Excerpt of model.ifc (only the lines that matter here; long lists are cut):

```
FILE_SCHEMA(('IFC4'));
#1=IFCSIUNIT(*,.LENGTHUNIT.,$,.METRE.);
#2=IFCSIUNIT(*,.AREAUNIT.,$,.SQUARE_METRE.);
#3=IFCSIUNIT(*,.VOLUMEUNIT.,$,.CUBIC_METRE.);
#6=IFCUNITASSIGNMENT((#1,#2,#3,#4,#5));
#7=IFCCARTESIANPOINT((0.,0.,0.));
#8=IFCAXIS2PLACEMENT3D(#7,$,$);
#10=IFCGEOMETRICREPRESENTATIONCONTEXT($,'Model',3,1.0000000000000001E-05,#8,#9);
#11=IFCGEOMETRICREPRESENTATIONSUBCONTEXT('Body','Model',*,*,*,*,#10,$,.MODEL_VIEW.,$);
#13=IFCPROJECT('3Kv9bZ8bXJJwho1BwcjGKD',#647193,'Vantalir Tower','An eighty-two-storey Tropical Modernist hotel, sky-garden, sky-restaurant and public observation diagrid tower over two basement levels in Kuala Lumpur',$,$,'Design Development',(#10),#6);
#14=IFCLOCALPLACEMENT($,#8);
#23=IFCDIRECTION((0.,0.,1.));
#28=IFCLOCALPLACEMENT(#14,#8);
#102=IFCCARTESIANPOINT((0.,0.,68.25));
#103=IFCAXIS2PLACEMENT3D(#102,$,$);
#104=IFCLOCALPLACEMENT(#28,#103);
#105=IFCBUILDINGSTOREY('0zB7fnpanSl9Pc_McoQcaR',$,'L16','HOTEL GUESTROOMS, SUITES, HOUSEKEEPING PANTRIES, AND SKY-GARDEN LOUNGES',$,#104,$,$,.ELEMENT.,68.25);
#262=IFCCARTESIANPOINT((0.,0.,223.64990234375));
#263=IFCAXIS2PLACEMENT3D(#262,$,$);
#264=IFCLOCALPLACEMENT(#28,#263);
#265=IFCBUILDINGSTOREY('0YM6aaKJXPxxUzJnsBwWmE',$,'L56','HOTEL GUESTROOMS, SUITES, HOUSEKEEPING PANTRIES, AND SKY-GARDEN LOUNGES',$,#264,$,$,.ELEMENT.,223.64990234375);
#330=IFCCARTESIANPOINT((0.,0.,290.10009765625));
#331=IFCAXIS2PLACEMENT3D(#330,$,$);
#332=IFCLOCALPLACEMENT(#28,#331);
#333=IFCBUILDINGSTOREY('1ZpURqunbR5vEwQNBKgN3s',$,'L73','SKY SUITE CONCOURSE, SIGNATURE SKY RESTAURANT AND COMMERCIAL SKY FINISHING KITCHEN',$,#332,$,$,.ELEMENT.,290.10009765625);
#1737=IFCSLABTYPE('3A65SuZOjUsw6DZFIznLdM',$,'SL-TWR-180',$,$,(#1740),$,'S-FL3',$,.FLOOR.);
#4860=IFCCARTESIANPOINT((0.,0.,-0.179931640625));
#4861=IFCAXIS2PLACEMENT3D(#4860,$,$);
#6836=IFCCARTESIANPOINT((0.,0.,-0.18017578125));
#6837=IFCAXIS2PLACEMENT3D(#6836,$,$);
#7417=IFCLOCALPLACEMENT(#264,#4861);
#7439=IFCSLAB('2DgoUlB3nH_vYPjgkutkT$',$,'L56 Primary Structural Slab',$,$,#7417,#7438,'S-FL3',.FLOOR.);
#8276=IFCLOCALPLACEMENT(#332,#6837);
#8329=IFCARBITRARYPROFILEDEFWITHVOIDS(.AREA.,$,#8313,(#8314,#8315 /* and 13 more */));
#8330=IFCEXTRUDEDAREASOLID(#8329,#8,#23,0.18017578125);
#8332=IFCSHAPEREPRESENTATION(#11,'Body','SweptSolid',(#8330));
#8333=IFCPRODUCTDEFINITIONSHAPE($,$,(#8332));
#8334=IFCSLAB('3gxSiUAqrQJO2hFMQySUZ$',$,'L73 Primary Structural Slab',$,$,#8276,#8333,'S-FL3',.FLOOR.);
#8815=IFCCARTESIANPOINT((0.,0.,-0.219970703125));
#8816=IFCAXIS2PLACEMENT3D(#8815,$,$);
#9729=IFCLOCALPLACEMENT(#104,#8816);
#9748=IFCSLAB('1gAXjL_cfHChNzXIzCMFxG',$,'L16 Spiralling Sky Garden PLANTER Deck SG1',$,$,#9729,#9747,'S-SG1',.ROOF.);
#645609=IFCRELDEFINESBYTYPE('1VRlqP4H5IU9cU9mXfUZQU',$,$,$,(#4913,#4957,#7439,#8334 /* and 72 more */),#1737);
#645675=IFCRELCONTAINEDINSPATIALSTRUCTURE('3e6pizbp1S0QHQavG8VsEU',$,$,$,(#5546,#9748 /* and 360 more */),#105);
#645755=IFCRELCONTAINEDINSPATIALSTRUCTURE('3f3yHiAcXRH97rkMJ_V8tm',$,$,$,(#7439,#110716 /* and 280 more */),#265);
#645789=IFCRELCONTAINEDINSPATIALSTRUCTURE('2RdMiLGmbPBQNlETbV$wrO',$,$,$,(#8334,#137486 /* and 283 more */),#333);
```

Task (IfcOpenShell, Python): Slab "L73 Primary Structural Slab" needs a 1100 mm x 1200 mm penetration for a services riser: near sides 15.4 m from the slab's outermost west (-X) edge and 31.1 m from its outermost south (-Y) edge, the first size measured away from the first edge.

```python
import numpy as np
import ifcopenshell
import ifcopenshell.api.feature
import ifcopenshell.api.geometry
import ifcopenshell.api.root
import ifcopenshell.geom
import ifcopenshell.util.placement
import ifcopenshell.util.representation
import ifcopenshell.util.shape
import ifcopenshell.util.unit

model = ifcopenshell.open("model.ifc")
unit_scale = ifcopenshell.util.unit.calculate_unit_scale(model)
settings = ifcopenshell.geom.settings()


def volume(element):
    """Net volume in cubic metres, openings subtracted."""
    shape = ifcopenshell.geom.create_shape(settings, element)
    return ifcopenshell.util.shape.get_volume(shape.geometry)


slab = model.by_guid("3gxSiUAqrQJO2hFMQySUZ$")
before = volume(slab)

# Extent in the slab's own axes, in metres. The edges named are its -X and -Y sides.
slab_shape = ifcopenshell.geom.create_shape(settings, slab)
vertices = ifcopenshell.util.shape.get_vertices(slab_shape.geometry)
x_min, y_min, bottom = vertices.min(axis=0)
top = vertices[:, 2].max()

opening = ifcopenshell.api.root.create_entity(model, ifc_class="IfcOpeningElement", name="Services riser opening", predefined_type="OPENING")
context = ifcopenshell.util.representation.get_context(model, "Model", "Body", "MODEL_VIEW")
width, depth = 1.1, 1.2
outline = [(0.0, 0.0), (width, 0.0), (width, depth), (0.0, depth), (0.0, 0.0)]
# Overshoot both faces by 50 mm so the cut is clean.
shape = ifcopenshell.api.geometry.add_slab_representation(
    model, context=context, depth=top - bottom + 0.1, polyline=outline
)
ifcopenshell.api.geometry.assign_representation(model, product=opening, representation=shape)

matrix = ifcopenshell.util.placement.get_local_placement(slab.ObjectPlacement)
matrix[:, 3] = matrix @ np.append(np.array([x_min + 15.4, y_min + 31.1, bottom - 0.05]) / unit_scale, 1.0)
ifcopenshell.api.geometry.edit_object_placement(model, product=opening, matrix=matrix, is_si=False)
ifcopenshell.api.feature.add_feature(model, feature=opening, element=slab)

after = volume(slab)

print(f"slab volume {before:.3f} -> {after:.3f} m3")

model.write("model_updated.ifc")
```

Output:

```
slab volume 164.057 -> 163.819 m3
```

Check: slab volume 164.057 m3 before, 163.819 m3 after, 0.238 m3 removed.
